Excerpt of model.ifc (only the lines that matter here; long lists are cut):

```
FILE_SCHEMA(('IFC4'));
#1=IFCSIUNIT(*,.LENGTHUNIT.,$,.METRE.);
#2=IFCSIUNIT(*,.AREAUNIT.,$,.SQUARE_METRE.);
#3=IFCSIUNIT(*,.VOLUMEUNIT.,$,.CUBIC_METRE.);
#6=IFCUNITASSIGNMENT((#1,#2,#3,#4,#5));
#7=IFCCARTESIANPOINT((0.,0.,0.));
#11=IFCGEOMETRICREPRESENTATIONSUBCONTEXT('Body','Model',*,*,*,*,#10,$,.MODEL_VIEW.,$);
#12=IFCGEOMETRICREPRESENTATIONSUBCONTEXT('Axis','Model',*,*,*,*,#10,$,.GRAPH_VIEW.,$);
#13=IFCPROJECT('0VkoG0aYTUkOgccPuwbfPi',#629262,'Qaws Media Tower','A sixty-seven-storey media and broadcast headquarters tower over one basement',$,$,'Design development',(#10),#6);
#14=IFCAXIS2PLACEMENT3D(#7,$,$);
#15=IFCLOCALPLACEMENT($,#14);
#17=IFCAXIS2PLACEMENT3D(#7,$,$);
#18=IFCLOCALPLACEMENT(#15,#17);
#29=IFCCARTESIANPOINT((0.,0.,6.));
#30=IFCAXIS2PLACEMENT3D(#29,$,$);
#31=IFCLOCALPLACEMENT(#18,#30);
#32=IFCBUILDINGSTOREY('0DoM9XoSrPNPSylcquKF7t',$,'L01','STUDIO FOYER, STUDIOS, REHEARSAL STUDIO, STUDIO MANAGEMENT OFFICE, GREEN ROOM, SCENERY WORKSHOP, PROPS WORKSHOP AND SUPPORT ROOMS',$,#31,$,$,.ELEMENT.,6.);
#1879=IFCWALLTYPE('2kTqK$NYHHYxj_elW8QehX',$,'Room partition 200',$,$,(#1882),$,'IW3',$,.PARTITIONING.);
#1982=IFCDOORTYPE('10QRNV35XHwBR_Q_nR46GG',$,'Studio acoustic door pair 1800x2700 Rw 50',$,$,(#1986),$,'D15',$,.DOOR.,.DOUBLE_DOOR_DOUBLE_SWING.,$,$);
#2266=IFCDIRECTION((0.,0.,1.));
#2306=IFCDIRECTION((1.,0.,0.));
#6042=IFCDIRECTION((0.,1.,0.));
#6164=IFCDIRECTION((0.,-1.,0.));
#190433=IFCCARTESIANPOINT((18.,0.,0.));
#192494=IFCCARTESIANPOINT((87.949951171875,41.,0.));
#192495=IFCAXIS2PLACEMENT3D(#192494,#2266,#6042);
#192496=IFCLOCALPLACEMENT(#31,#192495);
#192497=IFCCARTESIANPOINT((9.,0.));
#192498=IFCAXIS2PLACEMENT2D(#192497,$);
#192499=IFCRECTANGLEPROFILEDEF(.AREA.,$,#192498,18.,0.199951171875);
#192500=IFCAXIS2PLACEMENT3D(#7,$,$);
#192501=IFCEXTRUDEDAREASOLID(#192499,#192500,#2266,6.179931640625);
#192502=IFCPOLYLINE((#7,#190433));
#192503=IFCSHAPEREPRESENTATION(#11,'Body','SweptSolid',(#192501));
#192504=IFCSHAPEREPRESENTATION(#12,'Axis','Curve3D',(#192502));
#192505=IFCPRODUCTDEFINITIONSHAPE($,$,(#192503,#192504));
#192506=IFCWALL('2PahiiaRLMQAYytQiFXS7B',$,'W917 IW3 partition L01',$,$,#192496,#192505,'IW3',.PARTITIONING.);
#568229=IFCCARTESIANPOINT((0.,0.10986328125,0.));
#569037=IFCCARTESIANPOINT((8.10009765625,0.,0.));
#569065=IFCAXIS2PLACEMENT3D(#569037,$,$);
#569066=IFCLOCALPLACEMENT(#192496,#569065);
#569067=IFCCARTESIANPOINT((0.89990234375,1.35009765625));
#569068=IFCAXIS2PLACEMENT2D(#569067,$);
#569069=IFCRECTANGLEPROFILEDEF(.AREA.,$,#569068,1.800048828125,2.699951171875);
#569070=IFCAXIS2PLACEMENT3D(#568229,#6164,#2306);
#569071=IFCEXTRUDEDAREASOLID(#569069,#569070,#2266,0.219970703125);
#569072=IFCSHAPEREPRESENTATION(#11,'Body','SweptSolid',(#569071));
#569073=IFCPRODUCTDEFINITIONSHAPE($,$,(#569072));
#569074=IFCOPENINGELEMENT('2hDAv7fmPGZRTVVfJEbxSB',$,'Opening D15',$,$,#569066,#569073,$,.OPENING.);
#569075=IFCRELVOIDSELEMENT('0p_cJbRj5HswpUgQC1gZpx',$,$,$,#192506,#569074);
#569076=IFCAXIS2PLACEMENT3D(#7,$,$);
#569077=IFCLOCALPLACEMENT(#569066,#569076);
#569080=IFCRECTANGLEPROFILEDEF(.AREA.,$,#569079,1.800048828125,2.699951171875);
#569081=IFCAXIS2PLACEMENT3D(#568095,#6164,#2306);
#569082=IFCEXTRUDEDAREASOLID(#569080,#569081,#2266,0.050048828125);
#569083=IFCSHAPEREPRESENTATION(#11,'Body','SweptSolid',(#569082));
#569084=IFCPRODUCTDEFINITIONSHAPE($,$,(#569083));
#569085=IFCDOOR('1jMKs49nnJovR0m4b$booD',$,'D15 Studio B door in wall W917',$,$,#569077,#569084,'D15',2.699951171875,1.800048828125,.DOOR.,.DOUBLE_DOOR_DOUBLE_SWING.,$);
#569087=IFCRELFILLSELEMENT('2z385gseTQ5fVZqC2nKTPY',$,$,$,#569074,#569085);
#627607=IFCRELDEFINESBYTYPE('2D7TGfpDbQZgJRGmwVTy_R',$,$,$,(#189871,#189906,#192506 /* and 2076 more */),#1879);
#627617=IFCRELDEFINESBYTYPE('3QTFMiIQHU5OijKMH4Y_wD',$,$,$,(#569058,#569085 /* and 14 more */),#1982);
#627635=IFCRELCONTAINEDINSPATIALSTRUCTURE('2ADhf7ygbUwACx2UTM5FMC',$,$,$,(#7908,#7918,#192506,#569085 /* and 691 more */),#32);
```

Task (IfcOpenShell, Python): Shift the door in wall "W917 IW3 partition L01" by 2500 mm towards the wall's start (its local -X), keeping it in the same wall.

```python
import ifcopenshell
import ifcopenshell.api.geometry
import ifcopenshell.util.placement
import ifcopenshell.util.unit

model = ifcopenshell.open("model.ifc")
unit_scale = ifcopenshell.util.unit.calculate_unit_scale(model)

door = model.by_guid("1jMKs49nnJovR0m4b$booD")
opening = door.FillsVoids[0].RelatingOpeningElement
wall = opening.VoidsElements[0].RelatingBuildingElement

wall_matrix = ifcopenshell.util.placement.get_local_placement(wall.ObjectPlacement)
shift = wall_matrix[:3, 0] * -2.5 / unit_scale
before = ifcopenshell.util.placement.get_local_placement(door.ObjectPlacement)[:3, 3].copy()

# The door is placed relative to its opening, so it follows when the opening moves.
matrix = ifcopenshell.util.placement.get_local_placement(opening.ObjectPlacement)
matrix[:3, 3] += shift
ifcopenshell.api.geometry.edit_object_placement(
    model, product=opening, matrix=matrix, is_si=False, should_transform_children=True
)

after = ifcopenshell.util.placement.get_local_placement(door.ObjectPlacement)[:3, 3]
print("door moved by", (after - before).round(3) + 0.0)

model.write("model_edited.ifc")
```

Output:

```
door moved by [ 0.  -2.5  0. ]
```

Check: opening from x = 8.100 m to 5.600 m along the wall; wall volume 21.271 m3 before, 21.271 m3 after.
